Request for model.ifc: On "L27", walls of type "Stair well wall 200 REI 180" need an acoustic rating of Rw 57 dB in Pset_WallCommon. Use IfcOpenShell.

First a look at what the model holds.

```python
import ifcopenshell
import ifcopenshell.util.element

model = ifcopenshell.open("model.ifc")
print(model.schema)
storey = next(s for s in model.by_type("IfcBuildingStorey") if s.Name == "L27")
walls = [e for e in ifcopenshell.util.element.get_decomposition(storey) if e.is_a("IfcWall")]
seen = {}
for e in walls:
    element_type = ifcopenshell.util.element.get_type(e)
    key = (element_type.Name if element_type != e and element_type else None, ifcopenshell.util.element.get_pset(e, "Pset_WallCommon", "AcousticRating"))
    seen[key] = seen.get(key, 0) + 1
for (name, value), count in sorted(seen.items(), key=str):
    print(count, "x", name, "|", value)
```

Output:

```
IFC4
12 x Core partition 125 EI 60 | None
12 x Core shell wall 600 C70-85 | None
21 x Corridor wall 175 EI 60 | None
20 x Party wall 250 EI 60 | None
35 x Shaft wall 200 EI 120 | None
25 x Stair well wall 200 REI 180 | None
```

```python
import ifcopenshell
import ifcopenshell.api.pset
import ifcopenshell.util.element

model = ifcopenshell.open("model.ifc")

storey = next(s for s in model.by_type("IfcBuildingStorey") if s.Name == "L27")
walls = [e for e in ifcopenshell.util.element.get_decomposition(storey) if e.is_a("IfcWall")]

count = 0
for e in walls:
    element_type = ifcopenshell.util.element.get_type(e)
    if element_type in (None, e) or element_type.Name != "Stair well wall 200 REI 180":
        continue
    found = ifcopenshell.util.element.get_pset(e, "Pset_WallCommon", should_inherit=False)
    if found:
        pset = model.by_id(found["id"])
        if len(ifcopenshell.util.element.get_elements_by_pset(pset)) > 1:
            pset = ifcopenshell.api.pset.unshare_pset(model, products=[e], pset=pset)[0]
    else:
        pset = ifcopenshell.api.pset.add_pset(model, product=e, name="Pset_WallCommon")
    ifcopenshell.api.pset.edit_pset(model, pset=pset, properties={"AcousticRating": "Rw 57 dB"})
    count += 1

print(count, "walls updated")

model.write("model-out.ifc")
```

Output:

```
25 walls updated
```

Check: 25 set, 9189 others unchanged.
